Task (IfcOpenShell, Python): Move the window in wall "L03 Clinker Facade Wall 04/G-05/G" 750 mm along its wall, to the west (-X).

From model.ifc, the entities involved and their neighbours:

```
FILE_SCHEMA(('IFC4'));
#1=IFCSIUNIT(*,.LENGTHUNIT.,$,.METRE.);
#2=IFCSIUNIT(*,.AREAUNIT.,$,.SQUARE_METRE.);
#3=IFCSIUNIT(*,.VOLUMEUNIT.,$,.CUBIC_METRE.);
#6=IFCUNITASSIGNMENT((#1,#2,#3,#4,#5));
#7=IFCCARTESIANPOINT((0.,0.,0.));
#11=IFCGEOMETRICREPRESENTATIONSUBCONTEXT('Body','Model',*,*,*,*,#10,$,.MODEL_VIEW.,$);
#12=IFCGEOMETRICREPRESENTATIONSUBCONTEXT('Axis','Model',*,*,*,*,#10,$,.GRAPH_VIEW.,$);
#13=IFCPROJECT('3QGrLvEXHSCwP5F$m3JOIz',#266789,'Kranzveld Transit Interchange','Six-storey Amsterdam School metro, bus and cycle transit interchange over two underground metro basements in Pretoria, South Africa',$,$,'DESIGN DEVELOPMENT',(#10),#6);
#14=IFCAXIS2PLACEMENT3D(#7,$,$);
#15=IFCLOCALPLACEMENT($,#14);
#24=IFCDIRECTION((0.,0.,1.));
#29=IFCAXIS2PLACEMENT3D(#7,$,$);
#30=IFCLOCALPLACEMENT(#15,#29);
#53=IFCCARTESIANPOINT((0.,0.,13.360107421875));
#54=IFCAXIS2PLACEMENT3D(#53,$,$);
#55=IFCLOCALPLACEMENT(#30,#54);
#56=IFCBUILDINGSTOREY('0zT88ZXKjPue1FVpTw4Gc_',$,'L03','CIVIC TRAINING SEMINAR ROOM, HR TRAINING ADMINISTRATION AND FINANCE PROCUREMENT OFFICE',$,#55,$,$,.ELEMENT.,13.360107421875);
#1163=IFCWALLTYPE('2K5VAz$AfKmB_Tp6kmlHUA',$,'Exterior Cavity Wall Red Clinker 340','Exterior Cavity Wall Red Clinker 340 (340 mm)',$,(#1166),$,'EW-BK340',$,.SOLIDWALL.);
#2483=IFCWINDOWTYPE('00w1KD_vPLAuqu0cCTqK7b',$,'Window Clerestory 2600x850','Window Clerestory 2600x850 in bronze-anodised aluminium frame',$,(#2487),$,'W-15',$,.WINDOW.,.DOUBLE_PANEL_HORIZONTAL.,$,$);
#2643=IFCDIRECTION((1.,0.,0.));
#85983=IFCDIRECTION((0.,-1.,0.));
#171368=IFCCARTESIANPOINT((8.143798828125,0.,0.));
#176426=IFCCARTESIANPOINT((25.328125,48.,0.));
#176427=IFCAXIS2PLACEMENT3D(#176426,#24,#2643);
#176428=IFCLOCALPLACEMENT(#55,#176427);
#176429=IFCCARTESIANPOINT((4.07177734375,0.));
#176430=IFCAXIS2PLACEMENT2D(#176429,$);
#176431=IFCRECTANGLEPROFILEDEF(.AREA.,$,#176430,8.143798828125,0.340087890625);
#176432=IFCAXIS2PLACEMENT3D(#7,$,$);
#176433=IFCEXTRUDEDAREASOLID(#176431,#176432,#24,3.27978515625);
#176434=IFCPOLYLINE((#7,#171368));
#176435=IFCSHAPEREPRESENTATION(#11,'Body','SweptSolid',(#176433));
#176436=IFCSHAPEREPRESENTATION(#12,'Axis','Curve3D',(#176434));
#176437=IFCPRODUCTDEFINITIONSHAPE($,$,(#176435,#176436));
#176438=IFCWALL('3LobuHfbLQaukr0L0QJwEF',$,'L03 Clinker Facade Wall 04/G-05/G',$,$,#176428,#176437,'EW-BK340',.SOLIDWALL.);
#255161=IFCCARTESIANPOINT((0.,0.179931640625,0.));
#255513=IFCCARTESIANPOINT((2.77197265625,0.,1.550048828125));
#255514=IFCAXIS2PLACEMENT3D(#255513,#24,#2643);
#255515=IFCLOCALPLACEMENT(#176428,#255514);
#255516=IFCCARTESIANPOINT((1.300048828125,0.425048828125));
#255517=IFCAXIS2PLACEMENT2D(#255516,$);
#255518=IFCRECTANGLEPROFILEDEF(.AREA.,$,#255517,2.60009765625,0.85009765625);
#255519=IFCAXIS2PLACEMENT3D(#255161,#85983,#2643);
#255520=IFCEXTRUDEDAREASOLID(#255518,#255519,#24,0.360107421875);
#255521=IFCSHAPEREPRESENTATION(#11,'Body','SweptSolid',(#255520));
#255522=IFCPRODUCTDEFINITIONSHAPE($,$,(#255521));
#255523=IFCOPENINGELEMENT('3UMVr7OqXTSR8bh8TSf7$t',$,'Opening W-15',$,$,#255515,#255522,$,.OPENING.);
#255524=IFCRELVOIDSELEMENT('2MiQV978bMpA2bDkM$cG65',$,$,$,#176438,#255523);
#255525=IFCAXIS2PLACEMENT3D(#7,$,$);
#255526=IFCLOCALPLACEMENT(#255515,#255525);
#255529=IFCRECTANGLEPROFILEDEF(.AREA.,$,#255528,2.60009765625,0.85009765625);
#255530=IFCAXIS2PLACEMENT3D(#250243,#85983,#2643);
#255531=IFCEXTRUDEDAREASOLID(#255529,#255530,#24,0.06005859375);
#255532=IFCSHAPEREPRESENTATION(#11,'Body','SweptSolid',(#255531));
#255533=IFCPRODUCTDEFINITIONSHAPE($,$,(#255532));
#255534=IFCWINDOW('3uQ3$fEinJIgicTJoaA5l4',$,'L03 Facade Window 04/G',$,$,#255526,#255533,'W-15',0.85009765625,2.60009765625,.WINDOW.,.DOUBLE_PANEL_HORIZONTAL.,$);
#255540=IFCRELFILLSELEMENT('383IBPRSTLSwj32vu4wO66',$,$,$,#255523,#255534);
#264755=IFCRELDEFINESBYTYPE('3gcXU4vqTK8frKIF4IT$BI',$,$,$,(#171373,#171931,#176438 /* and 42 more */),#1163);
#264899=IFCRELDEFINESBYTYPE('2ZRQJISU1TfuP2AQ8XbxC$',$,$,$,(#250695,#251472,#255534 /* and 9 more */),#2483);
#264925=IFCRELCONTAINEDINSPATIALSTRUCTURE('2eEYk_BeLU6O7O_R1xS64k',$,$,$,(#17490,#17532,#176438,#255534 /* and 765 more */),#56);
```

```python
import ifcopenshell
import ifcopenshell.api.geometry
import ifcopenshell.util.placement
import ifcopenshell.util.unit

model = ifcopenshell.open("model.ifc")
unit_scale = ifcopenshell.util.unit.calculate_unit_scale(model)

window = model.by_guid("3uQ3$fEinJIgicTJoaA5l4")
opening = window.FillsVoids[0].RelatingOpeningElement
wall = opening.VoidsElements[0].RelatingBuildingElement

wall_matrix = ifcopenshell.util.placement.get_local_placement(wall.ObjectPlacement)
shift = wall_matrix[:3, 0] * -0.75 / unit_scale
before = ifcopenshell.util.placement.get_local_placement(window.ObjectPlacement)[:3, 3].copy()

# The window is placed relative to its opening, so it follows when the opening moves.
matrix = ifcopenshell.util.placement.get_local_placement(opening.ObjectPlacement)
matrix[:3, 3] += shift
ifcopenshell.api.geometry.edit_object_placement(
    model, product=opening, matrix=matrix, is_si=False, should_transform_children=True
)

after = ifcopenshell.util.placement.get_local_placement(window.ObjectPlacement)[:3, 3]
print("window moved by", (after - before).round(3) + 0.0)

model.write("model_rev.ifc")
```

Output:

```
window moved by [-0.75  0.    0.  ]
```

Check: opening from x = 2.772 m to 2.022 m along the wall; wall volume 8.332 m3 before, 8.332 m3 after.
